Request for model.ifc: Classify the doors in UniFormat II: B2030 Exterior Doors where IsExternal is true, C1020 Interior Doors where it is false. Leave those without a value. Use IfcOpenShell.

First a look at what the model holds.

```python
import ifcopenshell
import ifcopenshell.util.element

model = ifcopenshell.open("model.ifc")
print(model.schema)
print("classifications:", [c.Name for c in model.by_type("IfcClassification")])
values = [ifcopenshell.util.element.get_pset(e, "Pset_DoorCommon", "IsExternal") for e in model.by_type("IfcDoor")]
for value in (True, False, None):
    print("IsExternal", value, values.count(value))
```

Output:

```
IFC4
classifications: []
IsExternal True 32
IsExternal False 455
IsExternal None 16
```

```python
import ifcopenshell
import ifcopenshell.api.classification
import ifcopenshell.util.element

model = ifcopenshell.open("model.ifc")

system = ifcopenshell.api.classification.add_classification(model, classification="UniFormat II")

doors = model.by_type("IfcDoor")
external = {e: ifcopenshell.util.element.get_pset(e, "Pset_DoorCommon", "IsExternal") for e in doors}
for flag, code, name in ((True, "B2030", "Exterior Doors"), (False, "C1020", "Interior Doors")):
    products = [e for e in doors if external[e] is flag]
    ifcopenshell.api.classification.add_reference(
        model, products=products, classification=system, identification=code, name=name
    )
    print(code, len(products))

model.write("model_edited.ifc")
```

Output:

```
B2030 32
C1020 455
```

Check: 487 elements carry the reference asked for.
